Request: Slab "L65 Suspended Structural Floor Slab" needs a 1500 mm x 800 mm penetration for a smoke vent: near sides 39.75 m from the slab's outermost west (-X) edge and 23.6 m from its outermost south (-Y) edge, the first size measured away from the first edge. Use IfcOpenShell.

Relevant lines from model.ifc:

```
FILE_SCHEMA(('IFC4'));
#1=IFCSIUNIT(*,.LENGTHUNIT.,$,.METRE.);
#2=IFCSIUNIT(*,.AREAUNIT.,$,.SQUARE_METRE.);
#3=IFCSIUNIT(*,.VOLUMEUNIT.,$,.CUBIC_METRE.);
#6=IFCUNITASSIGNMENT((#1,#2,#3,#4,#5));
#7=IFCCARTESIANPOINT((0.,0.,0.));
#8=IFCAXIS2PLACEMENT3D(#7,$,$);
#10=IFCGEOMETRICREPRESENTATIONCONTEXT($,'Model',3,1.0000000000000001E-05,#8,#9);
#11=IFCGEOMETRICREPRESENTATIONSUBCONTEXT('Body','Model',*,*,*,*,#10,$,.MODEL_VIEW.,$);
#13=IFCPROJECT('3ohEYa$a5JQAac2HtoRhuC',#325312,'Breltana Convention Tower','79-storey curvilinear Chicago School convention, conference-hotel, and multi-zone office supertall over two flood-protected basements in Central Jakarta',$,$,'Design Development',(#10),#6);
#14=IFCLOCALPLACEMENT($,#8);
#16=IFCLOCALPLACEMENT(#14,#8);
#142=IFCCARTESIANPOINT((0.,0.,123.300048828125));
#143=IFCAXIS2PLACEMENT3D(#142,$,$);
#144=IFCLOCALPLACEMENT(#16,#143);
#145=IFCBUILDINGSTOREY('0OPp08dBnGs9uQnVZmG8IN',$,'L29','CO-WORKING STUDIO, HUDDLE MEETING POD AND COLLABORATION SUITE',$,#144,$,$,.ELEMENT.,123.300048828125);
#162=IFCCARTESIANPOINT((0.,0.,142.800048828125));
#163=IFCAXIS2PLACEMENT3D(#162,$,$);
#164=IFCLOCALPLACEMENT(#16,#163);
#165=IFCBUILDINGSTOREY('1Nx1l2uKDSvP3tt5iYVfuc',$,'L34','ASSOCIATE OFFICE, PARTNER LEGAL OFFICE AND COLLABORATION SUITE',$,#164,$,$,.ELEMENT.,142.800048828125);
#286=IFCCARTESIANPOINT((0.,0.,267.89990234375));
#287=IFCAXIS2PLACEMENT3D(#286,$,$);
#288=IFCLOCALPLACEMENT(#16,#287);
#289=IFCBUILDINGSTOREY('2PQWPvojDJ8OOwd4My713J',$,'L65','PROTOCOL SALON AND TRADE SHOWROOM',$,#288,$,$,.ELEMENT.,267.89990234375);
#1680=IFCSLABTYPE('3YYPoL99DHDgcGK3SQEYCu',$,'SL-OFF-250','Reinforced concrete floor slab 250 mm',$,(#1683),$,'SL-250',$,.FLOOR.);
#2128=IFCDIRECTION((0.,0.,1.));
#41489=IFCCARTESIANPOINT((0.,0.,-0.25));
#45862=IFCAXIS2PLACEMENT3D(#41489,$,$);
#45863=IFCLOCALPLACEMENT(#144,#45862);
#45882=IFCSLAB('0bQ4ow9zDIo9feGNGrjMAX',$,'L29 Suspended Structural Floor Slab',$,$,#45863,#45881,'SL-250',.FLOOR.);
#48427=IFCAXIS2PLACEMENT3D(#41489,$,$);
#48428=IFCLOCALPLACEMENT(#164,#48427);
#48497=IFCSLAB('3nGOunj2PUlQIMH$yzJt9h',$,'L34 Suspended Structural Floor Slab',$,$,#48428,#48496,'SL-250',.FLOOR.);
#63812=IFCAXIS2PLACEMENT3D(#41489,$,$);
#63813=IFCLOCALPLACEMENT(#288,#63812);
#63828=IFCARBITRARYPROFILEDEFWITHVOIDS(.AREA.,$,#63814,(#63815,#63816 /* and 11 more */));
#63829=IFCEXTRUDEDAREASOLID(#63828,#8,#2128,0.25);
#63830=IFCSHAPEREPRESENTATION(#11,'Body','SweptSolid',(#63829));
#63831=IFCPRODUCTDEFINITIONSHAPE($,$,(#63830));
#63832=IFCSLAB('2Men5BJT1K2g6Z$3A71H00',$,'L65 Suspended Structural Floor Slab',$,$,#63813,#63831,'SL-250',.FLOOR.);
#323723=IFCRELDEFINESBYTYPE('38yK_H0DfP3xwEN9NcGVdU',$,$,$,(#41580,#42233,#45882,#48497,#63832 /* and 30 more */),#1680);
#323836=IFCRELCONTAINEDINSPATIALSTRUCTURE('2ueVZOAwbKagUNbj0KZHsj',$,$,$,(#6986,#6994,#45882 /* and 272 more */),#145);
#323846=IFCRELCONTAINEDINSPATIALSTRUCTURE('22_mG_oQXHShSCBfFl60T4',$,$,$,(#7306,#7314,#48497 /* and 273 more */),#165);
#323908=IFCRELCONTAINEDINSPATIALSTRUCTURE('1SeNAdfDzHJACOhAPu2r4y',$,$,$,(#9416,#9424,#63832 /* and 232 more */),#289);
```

```python
import numpy as np
import ifcopenshell
import ifcopenshell.api.feature
import ifcopenshell.api.geometry
import ifcopenshell.api.root
import ifcopenshell.geom
import ifcopenshell.util.placement
import ifcopenshell.util.representation
import ifcopenshell.util.shape
import ifcopenshell.util.unit

model = ifcopenshell.open("model.ifc")
unit_scale = ifcopenshell.util.unit.calculate_unit_scale(model)
settings = ifcopenshell.geom.settings()


def volume(element):
    """Net volume in cubic metres, openings subtracted."""
    shape = ifcopenshell.geom.create_shape(settings, element)
    return ifcopenshell.util.shape.get_volume(shape.geometry)


slab = model.by_guid("2Men5BJT1K2g6Z$3A71H00")
before = volume(slab)

# Extent in the slab's own axes, in metres. The edges named are its -X and -Y sides.
slab_shape = ifcopenshell.geom.create_shape(settings, slab)
vertices = ifcopenshell.util.shape.get_vertices(slab_shape.geometry)
x_min, y_min, bottom = vertices.min(axis=0)
top = vertices[:, 2].max()

opening = ifcopenshell.api.root.create_entity(model, ifc_class="IfcOpeningElement", name="Smoke vent opening", predefined_type="OPENING")
context = ifcopenshell.util.representation.get_context(model, "Model", "Body", "MODEL_VIEW")
width, depth = 1.5, 0.8
outline = [(0.0, 0.0), (width, 0.0), (width, depth), (0.0, depth), (0.0, 0.0)]
# Overshoot both faces by 50 mm so the cut is clean.
shape = ifcopenshell.api.geometry.add_slab_representation(
    model, context=context, depth=top - bottom + 0.1, polyline=outline
)
ifcopenshell.api.geometry.assign_representation(model, product=opening, representation=shape)

matrix = ifcopenshell.util.placement.get_local_placement(slab.ObjectPlacement)
matrix[:, 3] = matrix @ np.append(np.array([x_min + 39.75, y_min + 23.6, bottom - 0.05]) / unit_scale, 1.0)
ifcopenshell.api.geometry.edit_object_placement(model, product=opening, matrix=matrix, is_si=False)
ifcopenshell.api.feature.add_feature(model, feature=opening, element=slab)

after = volume(slab)

print(f"slab volume {before:.3f} -> {after:.3f} m3")

model.write("model_rev.ifc")
```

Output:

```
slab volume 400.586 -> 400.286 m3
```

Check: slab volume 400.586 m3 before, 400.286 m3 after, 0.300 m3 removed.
